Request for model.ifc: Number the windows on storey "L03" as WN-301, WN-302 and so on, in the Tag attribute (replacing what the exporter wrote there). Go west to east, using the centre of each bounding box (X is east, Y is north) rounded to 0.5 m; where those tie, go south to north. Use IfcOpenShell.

First a look at what the model holds.

```python
import ifcopenshell
import ifcopenshell.util.element
import ifcopenshell.util.placement

model = ifcopenshell.open("model.ifc")
print(model.schema)
storey = next(s for s in model.by_type("IfcBuildingStorey") if s.Name == "L03")
windows = [e for e in ifcopenshell.util.element.get_decomposition(storey) if e.is_a("IfcWindow")]
for e in sorted(windows, key=lambda e: e.id()):
    origin = ifcopenshell.util.placement.get_local_placement(e.ObjectPlacement)[:3, 3]
    print(e.id(), e.Tag, e.Name, origin.round(2) + 0.0, sep=" | ")
```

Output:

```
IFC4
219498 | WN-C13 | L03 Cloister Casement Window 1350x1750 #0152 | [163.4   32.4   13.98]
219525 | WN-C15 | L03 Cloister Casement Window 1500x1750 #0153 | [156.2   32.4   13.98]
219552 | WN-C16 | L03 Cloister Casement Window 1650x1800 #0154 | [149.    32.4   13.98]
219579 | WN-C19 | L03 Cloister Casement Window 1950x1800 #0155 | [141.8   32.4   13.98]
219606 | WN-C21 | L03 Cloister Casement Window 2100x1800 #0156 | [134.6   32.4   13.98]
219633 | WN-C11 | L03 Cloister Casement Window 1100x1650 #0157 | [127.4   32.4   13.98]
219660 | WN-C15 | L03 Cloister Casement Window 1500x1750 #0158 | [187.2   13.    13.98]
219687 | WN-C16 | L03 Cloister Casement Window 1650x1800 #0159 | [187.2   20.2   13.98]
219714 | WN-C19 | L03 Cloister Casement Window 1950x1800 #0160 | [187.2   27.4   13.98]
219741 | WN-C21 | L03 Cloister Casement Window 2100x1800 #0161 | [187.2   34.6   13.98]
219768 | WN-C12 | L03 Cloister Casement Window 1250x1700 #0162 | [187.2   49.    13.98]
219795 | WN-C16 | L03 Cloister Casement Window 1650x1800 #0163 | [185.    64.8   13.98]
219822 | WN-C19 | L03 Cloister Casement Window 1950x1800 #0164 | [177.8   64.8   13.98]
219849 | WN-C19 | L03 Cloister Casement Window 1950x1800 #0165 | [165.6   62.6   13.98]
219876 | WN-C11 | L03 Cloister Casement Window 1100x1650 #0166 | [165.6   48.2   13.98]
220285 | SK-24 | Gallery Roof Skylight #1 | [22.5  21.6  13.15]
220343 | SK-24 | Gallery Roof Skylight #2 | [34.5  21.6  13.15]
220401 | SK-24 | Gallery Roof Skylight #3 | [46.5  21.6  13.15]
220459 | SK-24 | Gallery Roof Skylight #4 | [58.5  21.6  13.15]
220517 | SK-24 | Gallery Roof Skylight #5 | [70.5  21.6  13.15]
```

```python
import ifcopenshell
import ifcopenshell.geom
import ifcopenshell.util.element
import ifcopenshell.util.shape

model = ifcopenshell.open("model.ifc")
settings = ifcopenshell.geom.settings()
settings.set("use-world-coords", True)


def centre(element):
    shape = ifcopenshell.geom.create_shape(settings, element)
    return ifcopenshell.util.shape.get_bbox_centroid(shape.geometry)


storey = next(s for s in model.by_type("IfcBuildingStorey") if s.Name == "L03")
windows = [e for e in ifcopenshell.util.element.get_decomposition(storey) if e.is_a("IfcWindow")]

# Insertion points can sit at a corner or the storey origin, so sort by the geometry (in metres).
centres = {e: centre(e) for e in windows}
windows.sort(key=lambda e: (round(centres[e][0] / 0.5), centres[e][1]))

for i, e in enumerate(windows, start=1):
    number = f"WN-3{i:02d}"
    e.Tag = number
    print(e.id(), number)

model.write("model-out.ifc")
```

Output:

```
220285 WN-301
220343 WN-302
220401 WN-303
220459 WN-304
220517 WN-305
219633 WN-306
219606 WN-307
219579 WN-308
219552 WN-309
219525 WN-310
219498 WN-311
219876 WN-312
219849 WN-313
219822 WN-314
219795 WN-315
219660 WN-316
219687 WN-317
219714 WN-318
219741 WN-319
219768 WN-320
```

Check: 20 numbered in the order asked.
